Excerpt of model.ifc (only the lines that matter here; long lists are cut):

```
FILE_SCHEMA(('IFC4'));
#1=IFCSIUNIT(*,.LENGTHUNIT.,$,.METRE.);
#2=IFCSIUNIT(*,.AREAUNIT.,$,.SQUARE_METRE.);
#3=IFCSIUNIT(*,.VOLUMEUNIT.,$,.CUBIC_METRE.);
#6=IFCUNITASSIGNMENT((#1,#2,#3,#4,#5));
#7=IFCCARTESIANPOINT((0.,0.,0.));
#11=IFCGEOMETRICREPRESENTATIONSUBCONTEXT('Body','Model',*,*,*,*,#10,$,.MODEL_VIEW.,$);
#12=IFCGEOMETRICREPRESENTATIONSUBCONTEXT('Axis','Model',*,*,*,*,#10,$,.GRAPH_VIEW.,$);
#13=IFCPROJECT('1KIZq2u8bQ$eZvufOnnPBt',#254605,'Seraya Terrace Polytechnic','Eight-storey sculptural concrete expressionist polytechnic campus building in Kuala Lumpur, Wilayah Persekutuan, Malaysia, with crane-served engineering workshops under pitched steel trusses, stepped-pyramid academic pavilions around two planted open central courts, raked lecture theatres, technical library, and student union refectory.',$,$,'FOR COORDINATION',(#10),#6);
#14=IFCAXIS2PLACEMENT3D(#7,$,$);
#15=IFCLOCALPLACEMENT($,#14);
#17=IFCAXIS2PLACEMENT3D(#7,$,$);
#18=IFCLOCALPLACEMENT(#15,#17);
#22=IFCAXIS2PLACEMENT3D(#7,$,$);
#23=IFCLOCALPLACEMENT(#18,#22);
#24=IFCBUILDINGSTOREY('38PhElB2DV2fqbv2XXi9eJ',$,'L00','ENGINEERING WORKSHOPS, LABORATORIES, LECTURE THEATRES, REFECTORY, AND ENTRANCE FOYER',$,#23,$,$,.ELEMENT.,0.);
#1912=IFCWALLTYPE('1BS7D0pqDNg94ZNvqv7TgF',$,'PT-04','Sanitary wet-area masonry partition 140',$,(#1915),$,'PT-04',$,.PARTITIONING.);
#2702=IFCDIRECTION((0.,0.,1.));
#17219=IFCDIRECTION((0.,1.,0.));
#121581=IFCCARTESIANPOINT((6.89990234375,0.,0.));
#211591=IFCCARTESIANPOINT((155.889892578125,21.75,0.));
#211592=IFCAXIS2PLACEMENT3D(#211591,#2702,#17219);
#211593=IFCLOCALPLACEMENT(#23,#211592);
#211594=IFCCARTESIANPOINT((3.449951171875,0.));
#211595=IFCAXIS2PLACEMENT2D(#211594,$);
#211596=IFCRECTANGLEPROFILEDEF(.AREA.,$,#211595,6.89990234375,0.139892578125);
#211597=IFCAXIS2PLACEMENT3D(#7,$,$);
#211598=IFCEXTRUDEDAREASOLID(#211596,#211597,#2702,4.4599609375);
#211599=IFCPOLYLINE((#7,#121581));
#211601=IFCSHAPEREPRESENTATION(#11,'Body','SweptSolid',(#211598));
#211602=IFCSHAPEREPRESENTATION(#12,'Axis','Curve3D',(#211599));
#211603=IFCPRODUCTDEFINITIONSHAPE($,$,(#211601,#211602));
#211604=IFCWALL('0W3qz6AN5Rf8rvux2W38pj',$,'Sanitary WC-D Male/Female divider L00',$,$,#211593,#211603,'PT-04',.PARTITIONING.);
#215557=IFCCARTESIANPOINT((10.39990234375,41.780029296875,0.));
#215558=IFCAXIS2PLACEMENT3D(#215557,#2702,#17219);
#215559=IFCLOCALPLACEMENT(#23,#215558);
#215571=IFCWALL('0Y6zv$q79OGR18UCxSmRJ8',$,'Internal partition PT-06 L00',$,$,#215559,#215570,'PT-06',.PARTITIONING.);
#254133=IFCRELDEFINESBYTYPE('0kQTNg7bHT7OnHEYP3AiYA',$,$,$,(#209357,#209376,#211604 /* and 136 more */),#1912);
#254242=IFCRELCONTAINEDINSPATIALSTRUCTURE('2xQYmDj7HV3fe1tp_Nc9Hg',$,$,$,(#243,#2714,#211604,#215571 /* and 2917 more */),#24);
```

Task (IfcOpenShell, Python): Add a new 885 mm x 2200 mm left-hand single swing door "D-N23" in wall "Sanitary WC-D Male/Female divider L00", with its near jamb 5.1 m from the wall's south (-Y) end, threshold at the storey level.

```python
import numpy as np
import ifcopenshell
import ifcopenshell.api.feature
import ifcopenshell.api.geometry
import ifcopenshell.api.root
import ifcopenshell.api.spatial
import ifcopenshell.geom
import ifcopenshell.util.element
import ifcopenshell.util.placement
import ifcopenshell.util.representation
import ifcopenshell.util.shape
import ifcopenshell.util.unit

model = ifcopenshell.open("model.ifc")
unit_scale = ifcopenshell.util.unit.calculate_unit_scale(model)
settings = ifcopenshell.geom.settings()


def volume(element):
    """Net volume in cubic metres, openings subtracted."""
    shape = ifcopenshell.geom.create_shape(settings, element)
    return ifcopenshell.util.shape.get_volume(shape.geometry)


wall = model.by_guid("0W3qz6AN5Rf8rvux2W38pj")
storey = ifcopenshell.util.element.get_container(wall, ifc_class="IfcBuildingStorey")
context = ifcopenshell.util.representation.get_context(model, "Model", "Body", "MODEL_VIEW")
before = volume(wall)

width, height, from_end, sill = 0.885, 2.2, 5.1, 0.0  # metres

# The wall runs along its own X axis, and the end named is its -X end.
wall_shape = ifcopenshell.geom.create_shape(settings, wall)
x, y, z = ifcopenshell.util.shape.get_vertices(wall_shape.geometry).T
start = x.min() + from_end
face, thickness = float(y.min()), float(y.max() - y.min())
wall_matrix = ifcopenshell.util.placement.get_local_placement(wall.ObjectPlacement)
level = ifcopenshell.util.placement.get_local_placement(storey.ObjectPlacement)[2, 3]


def in_wall(x, y):
    """Placement at x, y metres in the wall's axes, at sill height."""
    matrix = wall_matrix.copy()
    matrix[:, 3] = wall_matrix @ np.array([x / unit_scale, y / unit_scale, 0.0, 1.0])
    matrix[2, 3] = level + sill / unit_scale
    return matrix


# Opening: a box that overshoots both wall faces by 50 mm.
opening = ifcopenshell.api.root.create_entity(model, ifc_class="IfcOpeningElement", predefined_type="OPENING")
box = ifcopenshell.api.geometry.add_wall_representation(
    model, context=context, length=width, height=height, thickness=thickness + 0.1
)
ifcopenshell.api.geometry.assign_representation(model, product=opening, representation=box)
ifcopenshell.api.geometry.edit_object_placement(model, product=opening, matrix=in_wall(start, face - 0.05), is_si=False)
ifcopenshell.api.feature.add_feature(model, feature=opening, element=wall)

door = ifcopenshell.api.root.create_entity(model, ifc_class="IfcDoor", name="D-N23", predefined_type="DOOR")
door.OverallWidth, door.OverallHeight = width / unit_scale, height / unit_scale
door.OperationType = "SINGLE_SWING_LEFT"
body = ifcopenshell.api.geometry.add_door_representation(
    model,
    context=context,
    overall_width=door.OverallWidth,
    overall_height=door.OverallHeight,
    operation_type="SINGLE_SWING_LEFT",
    lining_properties={"LiningDepth": thickness / unit_scale, "ThresholdDepth": thickness / unit_scale},
)
ifcopenshell.api.geometry.assign_representation(model, product=door, representation=body)
ifcopenshell.api.spatial.assign_container(model, products=[door], relating_structure=storey)
ifcopenshell.api.feature.add_filling(model, opening=opening, element=door)

# The lining spans the wall, so the door starts at the wall face.
ifcopenshell.api.geometry.edit_object_placement(model, product=door, matrix=in_wall(start, face), is_si=False)

after = volume(wall)

print(f"wall volume {before:.3f} -> {after:.3f} m3")

model.write("model_rev.ifc")
```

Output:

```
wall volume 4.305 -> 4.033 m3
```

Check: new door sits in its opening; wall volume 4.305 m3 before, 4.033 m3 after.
